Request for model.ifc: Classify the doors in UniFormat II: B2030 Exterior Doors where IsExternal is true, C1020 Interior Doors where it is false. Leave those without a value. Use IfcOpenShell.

First a look at what the model holds.

```python
import ifcopenshell
import ifcopenshell.util.element

model = ifcopenshell.open("model.ifc")
print(model.schema)
print("classifications:", [c.Name for c in model.by_type("IfcClassification")])
values = [ifcopenshell.util.element.get_pset(e, "Pset_DoorCommon", "IsExternal") for e in model.by_type("IfcDoor")]
for value in (True, False, None):
    print("IsExternal", value, values.count(value))
```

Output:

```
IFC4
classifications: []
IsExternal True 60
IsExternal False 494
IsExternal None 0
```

```python
import ifcopenshell
import ifcopenshell.api.classification
import ifcopenshell.util.element

model = ifcopenshell.open("model.ifc")

system = ifcopenshell.api.classification.add_classification(model, classification="UniFormat II")

doors = model.by_type("IfcDoor")
external = {e: ifcopenshell.util.element.get_pset(e, "Pset_DoorCommon", "IsExternal") for e in doors}
for flag, code, name in ((True, "B2030", "Exterior Doors"), (False, "C1020", "Interior Doors")):
    products = [e for e in doors if external[e] is flag]
    ifcopenshell.api.classification.add_reference(
        model, products=products, classification=system, identification=code, name=name
    )
    print(code, len(products))

model.write("model_updated.ifc")
```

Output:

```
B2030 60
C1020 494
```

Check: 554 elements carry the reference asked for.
